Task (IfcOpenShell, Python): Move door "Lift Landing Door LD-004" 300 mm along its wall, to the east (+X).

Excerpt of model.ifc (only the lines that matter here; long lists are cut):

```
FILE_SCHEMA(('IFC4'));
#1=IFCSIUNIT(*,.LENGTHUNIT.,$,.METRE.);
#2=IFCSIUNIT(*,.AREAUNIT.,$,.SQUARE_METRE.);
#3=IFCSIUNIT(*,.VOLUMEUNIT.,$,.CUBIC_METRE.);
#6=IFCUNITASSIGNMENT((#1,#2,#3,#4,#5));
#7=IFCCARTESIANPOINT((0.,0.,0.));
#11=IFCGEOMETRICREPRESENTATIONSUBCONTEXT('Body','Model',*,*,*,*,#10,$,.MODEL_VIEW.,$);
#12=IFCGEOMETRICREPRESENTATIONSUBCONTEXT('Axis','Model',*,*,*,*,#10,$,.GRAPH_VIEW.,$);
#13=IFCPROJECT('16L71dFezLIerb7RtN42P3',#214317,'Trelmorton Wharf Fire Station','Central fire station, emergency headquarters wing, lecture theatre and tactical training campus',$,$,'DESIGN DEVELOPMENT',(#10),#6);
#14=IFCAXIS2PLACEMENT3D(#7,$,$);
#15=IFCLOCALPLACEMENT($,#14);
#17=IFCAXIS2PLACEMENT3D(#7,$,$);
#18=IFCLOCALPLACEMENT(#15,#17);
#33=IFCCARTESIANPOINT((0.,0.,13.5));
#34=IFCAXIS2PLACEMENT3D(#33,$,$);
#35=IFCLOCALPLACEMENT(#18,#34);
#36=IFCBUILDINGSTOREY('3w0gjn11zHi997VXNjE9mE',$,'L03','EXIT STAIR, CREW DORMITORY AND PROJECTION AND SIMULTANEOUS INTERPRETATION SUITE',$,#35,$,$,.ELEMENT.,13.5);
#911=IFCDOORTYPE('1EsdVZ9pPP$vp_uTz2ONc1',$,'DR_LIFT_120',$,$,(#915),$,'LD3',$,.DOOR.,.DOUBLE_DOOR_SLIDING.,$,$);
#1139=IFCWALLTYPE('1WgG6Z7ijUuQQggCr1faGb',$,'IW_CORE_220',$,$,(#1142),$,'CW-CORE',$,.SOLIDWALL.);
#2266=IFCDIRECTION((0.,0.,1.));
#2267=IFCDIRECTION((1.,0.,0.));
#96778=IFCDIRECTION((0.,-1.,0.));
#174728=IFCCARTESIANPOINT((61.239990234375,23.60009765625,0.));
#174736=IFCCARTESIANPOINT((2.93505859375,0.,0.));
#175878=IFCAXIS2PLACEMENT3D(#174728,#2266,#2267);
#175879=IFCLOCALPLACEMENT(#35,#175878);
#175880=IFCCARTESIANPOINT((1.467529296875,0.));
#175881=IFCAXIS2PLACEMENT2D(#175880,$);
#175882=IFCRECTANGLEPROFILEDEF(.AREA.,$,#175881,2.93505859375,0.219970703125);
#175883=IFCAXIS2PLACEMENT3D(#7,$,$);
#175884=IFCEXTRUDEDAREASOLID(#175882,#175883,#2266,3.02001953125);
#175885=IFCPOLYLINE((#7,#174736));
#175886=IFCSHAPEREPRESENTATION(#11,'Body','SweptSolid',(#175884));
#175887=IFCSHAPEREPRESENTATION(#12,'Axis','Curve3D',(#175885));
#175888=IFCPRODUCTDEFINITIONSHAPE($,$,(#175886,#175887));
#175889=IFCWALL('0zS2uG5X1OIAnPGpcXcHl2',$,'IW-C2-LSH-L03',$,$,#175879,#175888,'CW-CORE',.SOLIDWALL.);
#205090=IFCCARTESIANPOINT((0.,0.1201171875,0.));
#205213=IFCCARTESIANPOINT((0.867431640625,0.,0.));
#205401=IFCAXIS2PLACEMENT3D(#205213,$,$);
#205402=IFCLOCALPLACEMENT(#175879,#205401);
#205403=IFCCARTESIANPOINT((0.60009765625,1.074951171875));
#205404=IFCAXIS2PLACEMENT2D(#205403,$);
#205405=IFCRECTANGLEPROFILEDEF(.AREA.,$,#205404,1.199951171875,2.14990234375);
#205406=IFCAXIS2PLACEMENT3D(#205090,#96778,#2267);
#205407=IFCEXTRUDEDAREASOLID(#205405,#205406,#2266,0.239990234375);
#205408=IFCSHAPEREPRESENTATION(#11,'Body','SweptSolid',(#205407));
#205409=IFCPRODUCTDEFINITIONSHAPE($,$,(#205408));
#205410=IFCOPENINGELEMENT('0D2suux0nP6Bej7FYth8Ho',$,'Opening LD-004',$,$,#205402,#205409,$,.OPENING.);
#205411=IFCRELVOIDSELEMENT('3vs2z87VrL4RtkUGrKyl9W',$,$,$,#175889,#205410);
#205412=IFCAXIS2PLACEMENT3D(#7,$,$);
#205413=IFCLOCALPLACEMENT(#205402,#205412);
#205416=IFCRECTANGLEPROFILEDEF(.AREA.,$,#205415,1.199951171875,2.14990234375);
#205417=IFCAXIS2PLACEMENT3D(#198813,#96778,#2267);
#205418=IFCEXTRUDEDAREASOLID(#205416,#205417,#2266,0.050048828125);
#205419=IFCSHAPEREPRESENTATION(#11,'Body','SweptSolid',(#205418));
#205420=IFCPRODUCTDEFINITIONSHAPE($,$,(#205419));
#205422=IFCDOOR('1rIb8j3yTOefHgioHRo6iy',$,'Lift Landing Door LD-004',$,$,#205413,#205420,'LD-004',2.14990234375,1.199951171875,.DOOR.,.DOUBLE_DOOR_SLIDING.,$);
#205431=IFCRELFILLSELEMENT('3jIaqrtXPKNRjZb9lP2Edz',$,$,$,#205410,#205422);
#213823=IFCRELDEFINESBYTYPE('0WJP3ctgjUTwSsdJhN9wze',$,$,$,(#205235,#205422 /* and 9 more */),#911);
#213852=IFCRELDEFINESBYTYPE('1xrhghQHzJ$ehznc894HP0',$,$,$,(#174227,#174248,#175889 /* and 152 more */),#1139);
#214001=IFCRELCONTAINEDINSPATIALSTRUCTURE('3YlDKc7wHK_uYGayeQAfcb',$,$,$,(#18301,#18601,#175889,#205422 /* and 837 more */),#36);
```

```python
import ifcopenshell
import ifcopenshell.api.geometry
import ifcopenshell.util.placement
import ifcopenshell.util.unit

model = ifcopenshell.open("model.ifc")
unit_scale = ifcopenshell.util.unit.calculate_unit_scale(model)

door = model.by_guid("1rIb8j3yTOefHgioHRo6iy")
opening = door.FillsVoids[0].RelatingOpeningElement
wall = opening.VoidsElements[0].RelatingBuildingElement

wall_matrix = ifcopenshell.util.placement.get_local_placement(wall.ObjectPlacement)
shift = wall_matrix[:3, 0] * 0.3 / unit_scale
before = ifcopenshell.util.placement.get_local_placement(door.ObjectPlacement)[:3, 3].copy()

# The door is placed relative to its opening, so it follows when the opening moves.
matrix = ifcopenshell.util.placement.get_local_placement(opening.ObjectPlacement)
matrix[:3, 3] += shift
ifcopenshell.api.geometry.edit_object_placement(
    model, product=opening, matrix=matrix, is_si=False, should_transform_children=True
)

after = ifcopenshell.util.placement.get_local_placement(door.ObjectPlacement)[:3, 3]
print("door moved by", (after - before).round(3) + 0.0)

model.write("model_updated.ifc")
```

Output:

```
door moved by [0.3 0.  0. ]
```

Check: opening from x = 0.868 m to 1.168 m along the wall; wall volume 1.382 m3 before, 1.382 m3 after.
